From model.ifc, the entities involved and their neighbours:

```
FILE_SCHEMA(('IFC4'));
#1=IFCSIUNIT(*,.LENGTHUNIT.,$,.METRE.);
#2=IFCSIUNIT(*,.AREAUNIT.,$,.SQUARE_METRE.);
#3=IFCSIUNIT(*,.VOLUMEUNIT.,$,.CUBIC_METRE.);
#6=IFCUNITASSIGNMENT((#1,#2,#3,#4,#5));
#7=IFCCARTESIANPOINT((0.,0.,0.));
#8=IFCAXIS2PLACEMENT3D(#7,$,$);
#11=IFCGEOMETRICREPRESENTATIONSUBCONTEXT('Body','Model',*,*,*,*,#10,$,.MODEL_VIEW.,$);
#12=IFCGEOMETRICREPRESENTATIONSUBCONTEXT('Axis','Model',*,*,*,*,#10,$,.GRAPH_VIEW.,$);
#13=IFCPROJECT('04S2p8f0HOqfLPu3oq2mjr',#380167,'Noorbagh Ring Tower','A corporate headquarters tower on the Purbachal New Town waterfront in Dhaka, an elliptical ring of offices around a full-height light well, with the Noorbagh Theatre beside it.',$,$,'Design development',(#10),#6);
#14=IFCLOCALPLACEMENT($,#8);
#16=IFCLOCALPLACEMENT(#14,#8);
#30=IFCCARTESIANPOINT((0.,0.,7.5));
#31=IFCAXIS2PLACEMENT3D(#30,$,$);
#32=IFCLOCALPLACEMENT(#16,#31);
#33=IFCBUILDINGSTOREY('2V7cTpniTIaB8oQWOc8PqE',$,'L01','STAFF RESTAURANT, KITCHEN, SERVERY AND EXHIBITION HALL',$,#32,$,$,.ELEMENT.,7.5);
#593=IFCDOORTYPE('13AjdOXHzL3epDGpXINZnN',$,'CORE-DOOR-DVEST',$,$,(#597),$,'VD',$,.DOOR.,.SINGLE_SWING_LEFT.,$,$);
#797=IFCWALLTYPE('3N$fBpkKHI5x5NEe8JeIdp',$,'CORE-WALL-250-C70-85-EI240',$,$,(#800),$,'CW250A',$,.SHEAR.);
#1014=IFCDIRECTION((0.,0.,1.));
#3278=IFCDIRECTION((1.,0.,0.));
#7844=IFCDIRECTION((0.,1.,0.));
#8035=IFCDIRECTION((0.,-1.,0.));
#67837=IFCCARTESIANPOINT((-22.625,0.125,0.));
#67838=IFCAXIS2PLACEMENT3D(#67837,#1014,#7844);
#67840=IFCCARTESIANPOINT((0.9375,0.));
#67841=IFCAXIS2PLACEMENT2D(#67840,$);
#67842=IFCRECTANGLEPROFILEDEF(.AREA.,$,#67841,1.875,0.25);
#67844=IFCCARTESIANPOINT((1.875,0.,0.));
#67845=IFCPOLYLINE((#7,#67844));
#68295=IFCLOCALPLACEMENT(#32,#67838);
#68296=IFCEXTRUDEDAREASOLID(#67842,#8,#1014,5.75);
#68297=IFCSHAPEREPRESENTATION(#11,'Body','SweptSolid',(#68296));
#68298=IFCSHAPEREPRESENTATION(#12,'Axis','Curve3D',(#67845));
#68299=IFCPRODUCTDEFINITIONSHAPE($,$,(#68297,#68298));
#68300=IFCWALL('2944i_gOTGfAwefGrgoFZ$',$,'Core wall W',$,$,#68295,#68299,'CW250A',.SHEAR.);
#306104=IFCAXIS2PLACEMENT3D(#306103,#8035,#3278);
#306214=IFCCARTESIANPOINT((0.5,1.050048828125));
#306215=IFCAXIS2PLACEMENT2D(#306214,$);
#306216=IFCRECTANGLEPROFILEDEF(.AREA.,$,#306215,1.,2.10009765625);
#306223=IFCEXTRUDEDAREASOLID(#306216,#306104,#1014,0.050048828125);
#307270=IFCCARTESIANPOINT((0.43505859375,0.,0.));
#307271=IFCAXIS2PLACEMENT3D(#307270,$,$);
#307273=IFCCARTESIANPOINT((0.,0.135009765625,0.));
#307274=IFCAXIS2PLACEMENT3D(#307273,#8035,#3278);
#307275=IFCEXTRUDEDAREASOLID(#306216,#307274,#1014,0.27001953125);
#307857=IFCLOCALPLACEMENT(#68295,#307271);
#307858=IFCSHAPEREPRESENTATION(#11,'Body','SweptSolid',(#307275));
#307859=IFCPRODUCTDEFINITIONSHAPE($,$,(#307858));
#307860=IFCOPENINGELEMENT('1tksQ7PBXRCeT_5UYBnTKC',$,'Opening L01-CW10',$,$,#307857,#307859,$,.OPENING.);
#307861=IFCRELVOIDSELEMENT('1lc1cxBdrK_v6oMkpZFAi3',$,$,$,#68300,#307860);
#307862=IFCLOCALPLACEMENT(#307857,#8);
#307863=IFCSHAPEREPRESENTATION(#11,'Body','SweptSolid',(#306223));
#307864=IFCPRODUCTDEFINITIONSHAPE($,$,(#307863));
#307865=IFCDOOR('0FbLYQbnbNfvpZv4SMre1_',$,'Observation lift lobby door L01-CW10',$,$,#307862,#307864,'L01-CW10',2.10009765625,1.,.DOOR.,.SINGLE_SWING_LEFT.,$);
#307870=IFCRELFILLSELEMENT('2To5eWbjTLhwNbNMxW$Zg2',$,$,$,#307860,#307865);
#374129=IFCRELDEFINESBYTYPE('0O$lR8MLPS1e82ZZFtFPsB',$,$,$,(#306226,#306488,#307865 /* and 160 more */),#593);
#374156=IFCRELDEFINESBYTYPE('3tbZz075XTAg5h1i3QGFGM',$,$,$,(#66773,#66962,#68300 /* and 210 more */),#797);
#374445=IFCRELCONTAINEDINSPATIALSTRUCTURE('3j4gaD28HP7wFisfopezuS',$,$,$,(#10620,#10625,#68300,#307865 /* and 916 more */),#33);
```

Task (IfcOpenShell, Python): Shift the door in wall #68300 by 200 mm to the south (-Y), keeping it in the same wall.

```python
import ifcopenshell
import ifcopenshell.api.geometry
import ifcopenshell.util.placement
import ifcopenshell.util.unit

model = ifcopenshell.open("model.ifc")
unit_scale = ifcopenshell.util.unit.calculate_unit_scale(model)

door = model.by_id(307865)
opening = door.FillsVoids[0].RelatingOpeningElement
wall = opening.VoidsElements[0].RelatingBuildingElement

wall_matrix = ifcopenshell.util.placement.get_local_placement(wall.ObjectPlacement)
shift = wall_matrix[:3, 0] * -0.2 / unit_scale
before = ifcopenshell.util.placement.get_local_placement(door.ObjectPlacement)[:3, 3].copy()

# The door is placed relative to its opening, so it follows when the opening moves.
matrix = ifcopenshell.util.placement.get_local_placement(opening.ObjectPlacement)
matrix[:3, 3] += shift
ifcopenshell.api.geometry.edit_object_placement(
    model, product=opening, matrix=matrix, is_si=False, should_transform_children=True
)

after = ifcopenshell.util.placement.get_local_placement(door.ObjectPlacement)[:3, 3]
print("door moved by", (after - before).round(3) + 0.0)

model.write("model_updated.ifc")
```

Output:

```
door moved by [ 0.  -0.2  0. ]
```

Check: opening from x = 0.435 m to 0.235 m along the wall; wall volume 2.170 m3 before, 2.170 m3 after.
